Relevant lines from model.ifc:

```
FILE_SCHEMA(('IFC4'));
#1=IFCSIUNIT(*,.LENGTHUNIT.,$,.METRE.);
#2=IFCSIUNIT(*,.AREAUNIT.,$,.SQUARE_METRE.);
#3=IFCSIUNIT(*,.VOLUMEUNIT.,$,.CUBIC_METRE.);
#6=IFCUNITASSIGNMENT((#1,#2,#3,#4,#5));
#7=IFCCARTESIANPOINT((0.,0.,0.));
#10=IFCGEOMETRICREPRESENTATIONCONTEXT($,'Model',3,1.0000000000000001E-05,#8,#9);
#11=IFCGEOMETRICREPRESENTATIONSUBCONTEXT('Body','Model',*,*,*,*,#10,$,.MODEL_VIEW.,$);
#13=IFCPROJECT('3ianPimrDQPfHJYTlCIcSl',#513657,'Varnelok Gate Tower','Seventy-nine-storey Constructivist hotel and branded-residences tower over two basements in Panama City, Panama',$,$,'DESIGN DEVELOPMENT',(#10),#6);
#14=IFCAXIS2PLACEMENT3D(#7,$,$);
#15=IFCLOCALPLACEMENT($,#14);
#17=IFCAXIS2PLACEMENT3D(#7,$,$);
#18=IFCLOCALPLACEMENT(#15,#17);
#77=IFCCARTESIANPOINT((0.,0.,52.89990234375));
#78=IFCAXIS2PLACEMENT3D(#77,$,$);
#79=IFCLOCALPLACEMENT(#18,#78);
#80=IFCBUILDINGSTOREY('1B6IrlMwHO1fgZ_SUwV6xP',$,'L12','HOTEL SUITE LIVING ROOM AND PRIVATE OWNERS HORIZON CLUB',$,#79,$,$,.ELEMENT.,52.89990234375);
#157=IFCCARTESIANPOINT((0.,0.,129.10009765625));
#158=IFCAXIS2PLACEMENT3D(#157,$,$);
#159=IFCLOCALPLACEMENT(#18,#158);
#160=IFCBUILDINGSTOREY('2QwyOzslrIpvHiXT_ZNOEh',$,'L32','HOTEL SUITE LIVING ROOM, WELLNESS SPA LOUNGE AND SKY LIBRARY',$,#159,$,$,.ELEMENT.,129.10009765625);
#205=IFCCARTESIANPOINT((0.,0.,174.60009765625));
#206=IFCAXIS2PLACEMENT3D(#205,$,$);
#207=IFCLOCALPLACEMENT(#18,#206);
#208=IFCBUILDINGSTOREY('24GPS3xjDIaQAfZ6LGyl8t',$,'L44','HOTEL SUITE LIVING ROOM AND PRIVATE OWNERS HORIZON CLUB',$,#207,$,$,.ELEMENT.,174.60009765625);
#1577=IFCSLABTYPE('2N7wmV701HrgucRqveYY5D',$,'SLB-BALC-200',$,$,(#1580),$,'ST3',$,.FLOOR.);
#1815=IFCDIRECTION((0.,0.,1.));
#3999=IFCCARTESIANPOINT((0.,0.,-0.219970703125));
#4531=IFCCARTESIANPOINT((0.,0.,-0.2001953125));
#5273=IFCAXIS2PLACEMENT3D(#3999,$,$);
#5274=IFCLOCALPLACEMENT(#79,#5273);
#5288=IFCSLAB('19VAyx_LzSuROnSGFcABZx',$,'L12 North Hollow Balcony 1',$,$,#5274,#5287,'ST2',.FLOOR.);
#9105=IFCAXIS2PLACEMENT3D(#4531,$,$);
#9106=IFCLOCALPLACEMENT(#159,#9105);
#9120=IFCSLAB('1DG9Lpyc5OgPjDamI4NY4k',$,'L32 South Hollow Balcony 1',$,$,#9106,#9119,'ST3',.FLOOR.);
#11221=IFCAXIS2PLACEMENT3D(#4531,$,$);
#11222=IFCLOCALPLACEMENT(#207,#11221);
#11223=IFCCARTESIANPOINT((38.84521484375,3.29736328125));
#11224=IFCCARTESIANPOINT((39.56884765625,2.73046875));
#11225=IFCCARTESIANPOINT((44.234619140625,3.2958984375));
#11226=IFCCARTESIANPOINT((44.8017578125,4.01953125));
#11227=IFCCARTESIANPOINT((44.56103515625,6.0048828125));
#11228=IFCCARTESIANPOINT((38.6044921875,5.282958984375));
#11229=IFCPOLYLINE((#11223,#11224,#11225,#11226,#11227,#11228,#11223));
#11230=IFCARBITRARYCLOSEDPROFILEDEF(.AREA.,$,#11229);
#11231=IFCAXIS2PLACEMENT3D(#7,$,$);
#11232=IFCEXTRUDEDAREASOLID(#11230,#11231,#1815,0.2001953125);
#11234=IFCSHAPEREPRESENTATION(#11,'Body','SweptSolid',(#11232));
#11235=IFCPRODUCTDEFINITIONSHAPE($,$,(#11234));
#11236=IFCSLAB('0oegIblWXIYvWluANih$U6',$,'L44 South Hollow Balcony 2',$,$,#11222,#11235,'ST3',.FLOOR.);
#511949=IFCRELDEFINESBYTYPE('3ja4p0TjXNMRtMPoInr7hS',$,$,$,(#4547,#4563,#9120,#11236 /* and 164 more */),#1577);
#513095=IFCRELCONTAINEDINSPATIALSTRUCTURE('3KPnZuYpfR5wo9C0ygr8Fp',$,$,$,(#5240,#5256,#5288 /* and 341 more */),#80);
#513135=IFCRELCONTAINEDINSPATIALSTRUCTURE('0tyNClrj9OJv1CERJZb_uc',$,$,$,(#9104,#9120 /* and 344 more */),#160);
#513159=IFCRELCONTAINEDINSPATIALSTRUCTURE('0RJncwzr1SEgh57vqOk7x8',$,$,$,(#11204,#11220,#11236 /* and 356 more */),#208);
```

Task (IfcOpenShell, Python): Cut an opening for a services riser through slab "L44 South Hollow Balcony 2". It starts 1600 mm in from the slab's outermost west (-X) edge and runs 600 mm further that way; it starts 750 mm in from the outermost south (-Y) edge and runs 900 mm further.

```python
import numpy as np
import ifcopenshell
import ifcopenshell.api.feature
import ifcopenshell.api.geometry
import ifcopenshell.api.root
import ifcopenshell.geom
import ifcopenshell.util.placement
import ifcopenshell.util.representation
import ifcopenshell.util.shape
import ifcopenshell.util.unit

model = ifcopenshell.open("model.ifc")
unit_scale = ifcopenshell.util.unit.calculate_unit_scale(model)
settings = ifcopenshell.geom.settings()


def volume(element):
    """Net volume in cubic metres, openings subtracted."""
    shape = ifcopenshell.geom.create_shape(settings, element)
    return ifcopenshell.util.shape.get_volume(shape.geometry)


slab = model.by_guid("0oegIblWXIYvWluANih$U6")
before = volume(slab)

# Extent in the slab's own axes, in metres. The edges named are its -X and -Y sides.
slab_shape = ifcopenshell.geom.create_shape(settings, slab)
vertices = ifcopenshell.util.shape.get_vertices(slab_shape.geometry)
x_min, y_min, bottom = vertices.min(axis=0)
top = vertices[:, 2].max()

opening = ifcopenshell.api.root.create_entity(model, ifc_class="IfcOpeningElement", name="Services riser opening", predefined_type="OPENING")
context = ifcopenshell.util.representation.get_context(model, "Model", "Body", "MODEL_VIEW")
width, depth = 0.6, 0.9
outline = [(0.0, 0.0), (width, 0.0), (width, depth), (0.0, depth), (0.0, 0.0)]
# Overshoot both faces by 50 mm so the cut is clean.
shape = ifcopenshell.api.geometry.add_slab_representation(
    model, context=context, depth=top - bottom + 0.1, polyline=outline
)
ifcopenshell.api.geometry.assign_representation(model, product=opening, representation=shape)

matrix = ifcopenshell.util.placement.get_local_placement(slab.ObjectPlacement)
matrix[:, 3] = matrix @ np.append(np.array([x_min + 1.6, y_min + 0.75, bottom - 0.05]) / unit_scale, 1.0)
ifcopenshell.api.geometry.edit_object_placement(model, product=opening, matrix=matrix, is_si=False)
ifcopenshell.api.feature.add_feature(model, feature=opening, element=slab)

after = volume(slab)

print(f"slab volume {before:.3f} -> {after:.3f} m3")

model.write("model_v2.ifc")
```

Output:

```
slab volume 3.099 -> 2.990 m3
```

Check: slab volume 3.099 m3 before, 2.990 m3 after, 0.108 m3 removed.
